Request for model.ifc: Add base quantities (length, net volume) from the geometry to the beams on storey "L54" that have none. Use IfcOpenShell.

First a look at what the model holds.

```python
import ifcopenshell
import ifcopenshell.util.element
import ifcopenshell.util.unit

model = ifcopenshell.open("model.ifc")
print(model.schema)
for unit_type in ("LENGTHUNIT", "AREAUNIT", "VOLUMEUNIT"):
    print(unit_type, ifcopenshell.util.unit.calculate_unit_scale(model, unit_type))
storey = next(s for s in model.by_type("IfcBuildingStorey") if s.Name == "L54")
beams = [e for e in ifcopenshell.util.element.get_decomposition(storey) if e.is_a("IfcBeam")]
for e in sorted(beams, key=lambda e: e.id()):
    print(e.id(), e.is_a(), e.Name, list(ifcopenshell.util.element.get_psets(e, qtos_only=True)), sep=" | ")
```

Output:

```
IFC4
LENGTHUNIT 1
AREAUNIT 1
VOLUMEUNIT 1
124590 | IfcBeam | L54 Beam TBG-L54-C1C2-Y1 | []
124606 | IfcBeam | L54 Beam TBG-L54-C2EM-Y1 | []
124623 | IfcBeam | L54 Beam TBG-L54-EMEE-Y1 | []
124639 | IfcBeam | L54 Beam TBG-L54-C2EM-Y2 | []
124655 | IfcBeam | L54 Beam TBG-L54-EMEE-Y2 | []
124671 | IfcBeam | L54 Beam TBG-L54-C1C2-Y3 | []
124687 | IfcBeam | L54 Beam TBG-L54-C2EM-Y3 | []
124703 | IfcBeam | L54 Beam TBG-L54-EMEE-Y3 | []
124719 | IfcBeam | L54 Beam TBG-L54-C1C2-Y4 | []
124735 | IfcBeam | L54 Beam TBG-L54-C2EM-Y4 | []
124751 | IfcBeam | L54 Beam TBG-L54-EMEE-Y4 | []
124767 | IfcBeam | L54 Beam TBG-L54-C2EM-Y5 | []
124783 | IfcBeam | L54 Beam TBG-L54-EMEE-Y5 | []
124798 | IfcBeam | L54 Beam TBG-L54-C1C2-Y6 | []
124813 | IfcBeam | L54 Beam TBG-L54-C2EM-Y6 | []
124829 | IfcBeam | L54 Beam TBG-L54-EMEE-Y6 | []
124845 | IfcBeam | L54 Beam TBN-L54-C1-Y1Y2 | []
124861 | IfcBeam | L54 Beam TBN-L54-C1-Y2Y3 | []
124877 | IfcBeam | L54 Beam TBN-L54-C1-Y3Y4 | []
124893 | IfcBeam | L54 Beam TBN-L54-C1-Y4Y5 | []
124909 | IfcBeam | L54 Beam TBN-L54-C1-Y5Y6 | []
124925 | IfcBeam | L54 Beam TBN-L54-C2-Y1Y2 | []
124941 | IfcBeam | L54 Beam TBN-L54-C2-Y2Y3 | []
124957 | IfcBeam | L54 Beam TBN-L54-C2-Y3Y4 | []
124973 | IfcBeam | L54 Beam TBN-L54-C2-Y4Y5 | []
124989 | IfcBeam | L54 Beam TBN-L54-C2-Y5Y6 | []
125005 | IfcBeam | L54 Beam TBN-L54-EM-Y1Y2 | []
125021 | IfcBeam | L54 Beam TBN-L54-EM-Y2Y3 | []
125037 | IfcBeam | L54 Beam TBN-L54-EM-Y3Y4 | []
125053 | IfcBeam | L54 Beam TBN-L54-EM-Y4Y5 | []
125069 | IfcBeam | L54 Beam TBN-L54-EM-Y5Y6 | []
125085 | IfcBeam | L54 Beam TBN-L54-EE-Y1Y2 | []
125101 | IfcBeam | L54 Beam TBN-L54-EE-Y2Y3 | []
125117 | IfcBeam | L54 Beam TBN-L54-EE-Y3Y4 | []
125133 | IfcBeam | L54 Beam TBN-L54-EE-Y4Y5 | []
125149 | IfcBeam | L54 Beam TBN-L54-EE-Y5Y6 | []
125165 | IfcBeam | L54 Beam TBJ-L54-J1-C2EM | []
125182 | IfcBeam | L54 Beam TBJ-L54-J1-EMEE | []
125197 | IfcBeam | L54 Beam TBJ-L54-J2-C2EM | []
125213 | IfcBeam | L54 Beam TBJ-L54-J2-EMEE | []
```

```python
import ifcopenshell
import ifcopenshell.api.pset
import ifcopenshell.geom
import ifcopenshell.util.element
import ifcopenshell.util.shape
import ifcopenshell.util.unit

model = ifcopenshell.open("model.ifc")
unit_scale = ifcopenshell.util.unit.calculate_unit_scale(model)
volume_scale = ifcopenshell.util.unit.calculate_unit_scale(model, "VOLUMEUNIT")
settings = ifcopenshell.geom.settings()

storey = next(s for s in model.by_type("IfcBuildingStorey") if s.Name == "L54")
beams = [e for e in ifcopenshell.util.element.get_decomposition(storey) if e.is_a("IfcBeam")]

for e in sorted(beams, key=lambda e: e.id()):
    if ifcopenshell.util.element.get_psets(e, qtos_only=True, should_inherit=False):
        continue
    # Geometry comes back in metres, in the element's own axes.
    shape = ifcopenshell.geom.create_shape(settings, e)
    values = {
        "Length": ifcopenshell.util.shape.get_max_xyz(shape.geometry) / unit_scale,
        "NetVolume": ifcopenshell.util.shape.get_volume(shape.geometry) / volume_scale,
    }
    qto = ifcopenshell.api.pset.add_qto(model, product=e, name="Qto_BeamBaseQuantities")
    ifcopenshell.api.pset.edit_qto(model, qto=qto, properties=values)
    print(e.id(), {k: round(v, 3) for k, v in values.items()})

model.write("model_v2.ifc")
```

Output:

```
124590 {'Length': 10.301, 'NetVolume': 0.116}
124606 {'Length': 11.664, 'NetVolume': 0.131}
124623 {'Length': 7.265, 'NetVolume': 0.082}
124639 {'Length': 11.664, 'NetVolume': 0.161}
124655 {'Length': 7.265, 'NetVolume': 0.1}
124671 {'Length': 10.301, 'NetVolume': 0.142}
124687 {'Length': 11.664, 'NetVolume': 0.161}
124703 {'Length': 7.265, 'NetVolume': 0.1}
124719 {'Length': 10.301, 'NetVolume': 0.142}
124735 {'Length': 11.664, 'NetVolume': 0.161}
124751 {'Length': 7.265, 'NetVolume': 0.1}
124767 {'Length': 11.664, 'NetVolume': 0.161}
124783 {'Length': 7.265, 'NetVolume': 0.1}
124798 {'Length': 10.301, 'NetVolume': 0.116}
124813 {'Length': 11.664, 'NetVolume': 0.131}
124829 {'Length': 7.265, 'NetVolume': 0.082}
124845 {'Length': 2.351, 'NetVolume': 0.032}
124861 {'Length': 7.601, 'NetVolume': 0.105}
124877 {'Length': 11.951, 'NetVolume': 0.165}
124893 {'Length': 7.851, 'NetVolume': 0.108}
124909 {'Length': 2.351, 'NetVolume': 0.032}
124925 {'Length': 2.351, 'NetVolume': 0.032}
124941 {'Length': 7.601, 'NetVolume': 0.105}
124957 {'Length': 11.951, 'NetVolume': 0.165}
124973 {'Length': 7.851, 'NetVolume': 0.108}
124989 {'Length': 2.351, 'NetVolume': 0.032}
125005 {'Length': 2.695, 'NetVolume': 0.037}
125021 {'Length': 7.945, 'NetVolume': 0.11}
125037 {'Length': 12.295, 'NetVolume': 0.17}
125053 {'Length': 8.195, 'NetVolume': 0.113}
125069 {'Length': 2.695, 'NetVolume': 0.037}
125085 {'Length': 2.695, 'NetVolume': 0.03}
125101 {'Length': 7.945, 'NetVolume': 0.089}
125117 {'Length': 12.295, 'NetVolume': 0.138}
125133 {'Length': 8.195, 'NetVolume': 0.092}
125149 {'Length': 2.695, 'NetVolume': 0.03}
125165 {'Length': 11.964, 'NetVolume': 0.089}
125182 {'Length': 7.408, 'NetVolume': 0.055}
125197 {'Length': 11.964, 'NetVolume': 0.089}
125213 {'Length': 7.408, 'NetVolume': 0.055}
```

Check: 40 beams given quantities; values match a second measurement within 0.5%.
